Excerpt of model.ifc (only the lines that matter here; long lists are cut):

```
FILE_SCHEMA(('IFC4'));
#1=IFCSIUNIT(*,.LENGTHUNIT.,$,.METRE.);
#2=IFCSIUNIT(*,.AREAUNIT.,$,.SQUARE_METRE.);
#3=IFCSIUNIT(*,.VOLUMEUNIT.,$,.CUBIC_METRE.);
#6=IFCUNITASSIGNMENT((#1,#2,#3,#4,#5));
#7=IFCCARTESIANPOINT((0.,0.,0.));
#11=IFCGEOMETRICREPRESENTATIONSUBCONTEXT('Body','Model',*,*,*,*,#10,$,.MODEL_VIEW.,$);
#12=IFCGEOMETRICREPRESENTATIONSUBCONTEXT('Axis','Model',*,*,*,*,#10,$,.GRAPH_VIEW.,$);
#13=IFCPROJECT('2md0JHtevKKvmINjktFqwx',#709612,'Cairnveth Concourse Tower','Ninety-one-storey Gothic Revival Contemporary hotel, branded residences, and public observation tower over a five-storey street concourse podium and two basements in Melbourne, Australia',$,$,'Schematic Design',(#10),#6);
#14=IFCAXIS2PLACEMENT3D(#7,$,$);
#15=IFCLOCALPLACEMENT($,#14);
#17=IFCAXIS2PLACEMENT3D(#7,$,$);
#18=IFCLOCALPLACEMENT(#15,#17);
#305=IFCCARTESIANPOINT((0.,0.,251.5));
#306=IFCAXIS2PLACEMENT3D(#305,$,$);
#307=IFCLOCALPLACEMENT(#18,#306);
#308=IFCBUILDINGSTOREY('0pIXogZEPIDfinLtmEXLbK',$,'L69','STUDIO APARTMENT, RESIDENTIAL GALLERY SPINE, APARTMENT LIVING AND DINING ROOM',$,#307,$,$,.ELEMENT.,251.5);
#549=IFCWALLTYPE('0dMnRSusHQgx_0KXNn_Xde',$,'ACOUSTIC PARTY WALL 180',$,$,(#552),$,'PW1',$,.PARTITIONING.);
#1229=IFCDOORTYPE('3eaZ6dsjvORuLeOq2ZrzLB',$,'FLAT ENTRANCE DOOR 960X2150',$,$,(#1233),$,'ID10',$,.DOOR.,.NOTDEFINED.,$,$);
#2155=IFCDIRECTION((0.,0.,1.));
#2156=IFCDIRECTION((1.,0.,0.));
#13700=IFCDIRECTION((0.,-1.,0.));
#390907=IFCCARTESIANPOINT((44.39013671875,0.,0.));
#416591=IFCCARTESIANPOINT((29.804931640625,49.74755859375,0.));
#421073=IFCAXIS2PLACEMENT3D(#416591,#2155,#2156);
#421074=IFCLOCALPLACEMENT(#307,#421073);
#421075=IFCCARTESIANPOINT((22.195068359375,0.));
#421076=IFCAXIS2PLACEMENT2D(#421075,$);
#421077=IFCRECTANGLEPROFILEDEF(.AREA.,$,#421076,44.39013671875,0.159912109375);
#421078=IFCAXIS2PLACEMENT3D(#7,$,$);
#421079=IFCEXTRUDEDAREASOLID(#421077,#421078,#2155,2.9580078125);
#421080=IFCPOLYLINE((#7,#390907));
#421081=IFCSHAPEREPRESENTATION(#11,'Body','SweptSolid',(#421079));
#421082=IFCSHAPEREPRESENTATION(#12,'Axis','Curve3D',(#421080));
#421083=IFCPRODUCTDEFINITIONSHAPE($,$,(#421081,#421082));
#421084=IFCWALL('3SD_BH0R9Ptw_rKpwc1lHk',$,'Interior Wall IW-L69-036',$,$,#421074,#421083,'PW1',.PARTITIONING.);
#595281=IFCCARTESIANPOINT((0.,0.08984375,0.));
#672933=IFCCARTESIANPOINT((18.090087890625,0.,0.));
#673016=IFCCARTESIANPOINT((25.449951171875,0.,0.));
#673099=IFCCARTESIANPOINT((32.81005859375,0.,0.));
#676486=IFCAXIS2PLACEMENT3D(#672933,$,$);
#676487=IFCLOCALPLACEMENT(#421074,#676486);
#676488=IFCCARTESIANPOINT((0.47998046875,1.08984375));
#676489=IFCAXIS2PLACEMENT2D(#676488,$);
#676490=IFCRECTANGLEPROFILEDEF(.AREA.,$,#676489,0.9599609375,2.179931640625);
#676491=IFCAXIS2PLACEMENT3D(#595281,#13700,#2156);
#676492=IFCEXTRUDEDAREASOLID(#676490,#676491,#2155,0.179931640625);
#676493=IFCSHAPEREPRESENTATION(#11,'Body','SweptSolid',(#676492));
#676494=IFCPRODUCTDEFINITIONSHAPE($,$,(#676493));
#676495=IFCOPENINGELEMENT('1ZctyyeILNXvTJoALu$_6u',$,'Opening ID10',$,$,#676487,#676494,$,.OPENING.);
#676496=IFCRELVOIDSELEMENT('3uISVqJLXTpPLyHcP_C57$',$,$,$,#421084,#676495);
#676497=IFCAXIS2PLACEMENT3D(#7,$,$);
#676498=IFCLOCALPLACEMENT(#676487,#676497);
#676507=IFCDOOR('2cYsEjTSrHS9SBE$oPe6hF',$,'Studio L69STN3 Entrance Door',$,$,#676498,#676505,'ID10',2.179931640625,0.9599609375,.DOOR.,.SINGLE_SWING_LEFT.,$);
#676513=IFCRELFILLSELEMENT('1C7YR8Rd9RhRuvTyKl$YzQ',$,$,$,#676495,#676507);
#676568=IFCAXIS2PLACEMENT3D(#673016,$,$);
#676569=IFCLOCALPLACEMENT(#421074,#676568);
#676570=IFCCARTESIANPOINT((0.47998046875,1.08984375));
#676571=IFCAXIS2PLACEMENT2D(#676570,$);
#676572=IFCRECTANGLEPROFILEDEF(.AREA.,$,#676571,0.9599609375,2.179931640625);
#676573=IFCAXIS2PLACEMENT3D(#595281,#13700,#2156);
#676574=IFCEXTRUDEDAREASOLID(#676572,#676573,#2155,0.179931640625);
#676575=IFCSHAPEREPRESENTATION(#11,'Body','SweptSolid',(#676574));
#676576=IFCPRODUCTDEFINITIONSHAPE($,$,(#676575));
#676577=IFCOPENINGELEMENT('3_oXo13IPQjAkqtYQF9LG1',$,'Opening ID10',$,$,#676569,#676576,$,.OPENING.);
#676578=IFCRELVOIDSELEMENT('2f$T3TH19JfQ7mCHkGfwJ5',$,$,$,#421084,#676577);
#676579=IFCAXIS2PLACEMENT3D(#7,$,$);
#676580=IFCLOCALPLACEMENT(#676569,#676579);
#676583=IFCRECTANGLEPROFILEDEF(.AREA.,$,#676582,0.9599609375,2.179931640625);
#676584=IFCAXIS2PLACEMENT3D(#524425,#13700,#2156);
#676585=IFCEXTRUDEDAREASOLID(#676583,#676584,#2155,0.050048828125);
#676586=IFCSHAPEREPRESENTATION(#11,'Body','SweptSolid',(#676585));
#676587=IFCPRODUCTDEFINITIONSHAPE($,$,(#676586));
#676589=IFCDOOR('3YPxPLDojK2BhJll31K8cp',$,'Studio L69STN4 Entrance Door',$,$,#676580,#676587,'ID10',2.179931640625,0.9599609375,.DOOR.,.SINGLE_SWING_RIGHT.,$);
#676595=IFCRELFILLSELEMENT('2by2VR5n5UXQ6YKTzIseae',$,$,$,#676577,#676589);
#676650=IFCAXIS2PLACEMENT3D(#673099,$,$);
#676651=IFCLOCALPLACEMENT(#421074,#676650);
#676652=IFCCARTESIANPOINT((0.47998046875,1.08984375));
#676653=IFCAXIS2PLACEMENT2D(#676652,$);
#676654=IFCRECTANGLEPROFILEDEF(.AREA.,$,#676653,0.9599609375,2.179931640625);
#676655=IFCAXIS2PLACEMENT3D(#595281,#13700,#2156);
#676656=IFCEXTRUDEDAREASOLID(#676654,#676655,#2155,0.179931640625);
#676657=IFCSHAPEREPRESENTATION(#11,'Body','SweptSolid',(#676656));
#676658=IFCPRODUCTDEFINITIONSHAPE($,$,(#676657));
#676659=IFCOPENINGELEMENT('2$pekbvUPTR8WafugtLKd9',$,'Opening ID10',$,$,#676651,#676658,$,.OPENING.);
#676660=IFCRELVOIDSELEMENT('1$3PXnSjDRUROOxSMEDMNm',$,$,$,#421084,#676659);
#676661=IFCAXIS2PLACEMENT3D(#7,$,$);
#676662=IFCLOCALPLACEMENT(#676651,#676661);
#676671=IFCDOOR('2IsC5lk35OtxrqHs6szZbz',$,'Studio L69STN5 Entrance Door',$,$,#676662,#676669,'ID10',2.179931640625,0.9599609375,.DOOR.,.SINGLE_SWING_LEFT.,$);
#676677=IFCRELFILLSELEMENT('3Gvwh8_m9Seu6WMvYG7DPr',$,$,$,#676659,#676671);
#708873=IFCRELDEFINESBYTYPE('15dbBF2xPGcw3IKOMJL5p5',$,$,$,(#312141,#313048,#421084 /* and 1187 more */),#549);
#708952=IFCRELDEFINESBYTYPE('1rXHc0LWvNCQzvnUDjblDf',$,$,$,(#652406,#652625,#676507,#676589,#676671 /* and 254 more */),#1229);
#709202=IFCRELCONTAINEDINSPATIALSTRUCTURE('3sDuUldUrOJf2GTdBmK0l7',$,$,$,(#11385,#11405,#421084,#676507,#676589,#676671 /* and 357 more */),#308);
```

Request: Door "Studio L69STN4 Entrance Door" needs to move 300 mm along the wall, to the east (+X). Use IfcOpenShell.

```python
import ifcopenshell
import ifcopenshell.api.geometry
import ifcopenshell.util.placement

model = ifcopenshell.open("model.ifc")

door = model.by_id(676589)
opening = door.FillsVoids[0].RelatingOpeningElement
wall = opening.VoidsElements[0].RelatingBuildingElement

wall_matrix = ifcopenshell.util.placement.get_local_placement(wall.ObjectPlacement)
shift = wall_matrix[:3, 0] * 0.3
before = ifcopenshell.util.placement.get_local_placement(door.ObjectPlacement)[:3, 3].copy()

# The door is placed relative to its opening, so it follows when the opening moves.
matrix = ifcopenshell.util.placement.get_local_placement(opening.ObjectPlacement)
matrix[:3, 3] += shift
ifcopenshell.api.geometry.edit_object_placement(
    model, product=opening, matrix=matrix, is_si=False, should_transform_children=True
)

after = ifcopenshell.util.placement.get_local_placement(door.ObjectPlacement)[:3, 3]
print("door moved by", (after - before).round(3) + 0.0)

model.write("model_edited.ifc")
```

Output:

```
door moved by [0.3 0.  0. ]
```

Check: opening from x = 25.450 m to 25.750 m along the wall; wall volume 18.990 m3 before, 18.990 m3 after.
